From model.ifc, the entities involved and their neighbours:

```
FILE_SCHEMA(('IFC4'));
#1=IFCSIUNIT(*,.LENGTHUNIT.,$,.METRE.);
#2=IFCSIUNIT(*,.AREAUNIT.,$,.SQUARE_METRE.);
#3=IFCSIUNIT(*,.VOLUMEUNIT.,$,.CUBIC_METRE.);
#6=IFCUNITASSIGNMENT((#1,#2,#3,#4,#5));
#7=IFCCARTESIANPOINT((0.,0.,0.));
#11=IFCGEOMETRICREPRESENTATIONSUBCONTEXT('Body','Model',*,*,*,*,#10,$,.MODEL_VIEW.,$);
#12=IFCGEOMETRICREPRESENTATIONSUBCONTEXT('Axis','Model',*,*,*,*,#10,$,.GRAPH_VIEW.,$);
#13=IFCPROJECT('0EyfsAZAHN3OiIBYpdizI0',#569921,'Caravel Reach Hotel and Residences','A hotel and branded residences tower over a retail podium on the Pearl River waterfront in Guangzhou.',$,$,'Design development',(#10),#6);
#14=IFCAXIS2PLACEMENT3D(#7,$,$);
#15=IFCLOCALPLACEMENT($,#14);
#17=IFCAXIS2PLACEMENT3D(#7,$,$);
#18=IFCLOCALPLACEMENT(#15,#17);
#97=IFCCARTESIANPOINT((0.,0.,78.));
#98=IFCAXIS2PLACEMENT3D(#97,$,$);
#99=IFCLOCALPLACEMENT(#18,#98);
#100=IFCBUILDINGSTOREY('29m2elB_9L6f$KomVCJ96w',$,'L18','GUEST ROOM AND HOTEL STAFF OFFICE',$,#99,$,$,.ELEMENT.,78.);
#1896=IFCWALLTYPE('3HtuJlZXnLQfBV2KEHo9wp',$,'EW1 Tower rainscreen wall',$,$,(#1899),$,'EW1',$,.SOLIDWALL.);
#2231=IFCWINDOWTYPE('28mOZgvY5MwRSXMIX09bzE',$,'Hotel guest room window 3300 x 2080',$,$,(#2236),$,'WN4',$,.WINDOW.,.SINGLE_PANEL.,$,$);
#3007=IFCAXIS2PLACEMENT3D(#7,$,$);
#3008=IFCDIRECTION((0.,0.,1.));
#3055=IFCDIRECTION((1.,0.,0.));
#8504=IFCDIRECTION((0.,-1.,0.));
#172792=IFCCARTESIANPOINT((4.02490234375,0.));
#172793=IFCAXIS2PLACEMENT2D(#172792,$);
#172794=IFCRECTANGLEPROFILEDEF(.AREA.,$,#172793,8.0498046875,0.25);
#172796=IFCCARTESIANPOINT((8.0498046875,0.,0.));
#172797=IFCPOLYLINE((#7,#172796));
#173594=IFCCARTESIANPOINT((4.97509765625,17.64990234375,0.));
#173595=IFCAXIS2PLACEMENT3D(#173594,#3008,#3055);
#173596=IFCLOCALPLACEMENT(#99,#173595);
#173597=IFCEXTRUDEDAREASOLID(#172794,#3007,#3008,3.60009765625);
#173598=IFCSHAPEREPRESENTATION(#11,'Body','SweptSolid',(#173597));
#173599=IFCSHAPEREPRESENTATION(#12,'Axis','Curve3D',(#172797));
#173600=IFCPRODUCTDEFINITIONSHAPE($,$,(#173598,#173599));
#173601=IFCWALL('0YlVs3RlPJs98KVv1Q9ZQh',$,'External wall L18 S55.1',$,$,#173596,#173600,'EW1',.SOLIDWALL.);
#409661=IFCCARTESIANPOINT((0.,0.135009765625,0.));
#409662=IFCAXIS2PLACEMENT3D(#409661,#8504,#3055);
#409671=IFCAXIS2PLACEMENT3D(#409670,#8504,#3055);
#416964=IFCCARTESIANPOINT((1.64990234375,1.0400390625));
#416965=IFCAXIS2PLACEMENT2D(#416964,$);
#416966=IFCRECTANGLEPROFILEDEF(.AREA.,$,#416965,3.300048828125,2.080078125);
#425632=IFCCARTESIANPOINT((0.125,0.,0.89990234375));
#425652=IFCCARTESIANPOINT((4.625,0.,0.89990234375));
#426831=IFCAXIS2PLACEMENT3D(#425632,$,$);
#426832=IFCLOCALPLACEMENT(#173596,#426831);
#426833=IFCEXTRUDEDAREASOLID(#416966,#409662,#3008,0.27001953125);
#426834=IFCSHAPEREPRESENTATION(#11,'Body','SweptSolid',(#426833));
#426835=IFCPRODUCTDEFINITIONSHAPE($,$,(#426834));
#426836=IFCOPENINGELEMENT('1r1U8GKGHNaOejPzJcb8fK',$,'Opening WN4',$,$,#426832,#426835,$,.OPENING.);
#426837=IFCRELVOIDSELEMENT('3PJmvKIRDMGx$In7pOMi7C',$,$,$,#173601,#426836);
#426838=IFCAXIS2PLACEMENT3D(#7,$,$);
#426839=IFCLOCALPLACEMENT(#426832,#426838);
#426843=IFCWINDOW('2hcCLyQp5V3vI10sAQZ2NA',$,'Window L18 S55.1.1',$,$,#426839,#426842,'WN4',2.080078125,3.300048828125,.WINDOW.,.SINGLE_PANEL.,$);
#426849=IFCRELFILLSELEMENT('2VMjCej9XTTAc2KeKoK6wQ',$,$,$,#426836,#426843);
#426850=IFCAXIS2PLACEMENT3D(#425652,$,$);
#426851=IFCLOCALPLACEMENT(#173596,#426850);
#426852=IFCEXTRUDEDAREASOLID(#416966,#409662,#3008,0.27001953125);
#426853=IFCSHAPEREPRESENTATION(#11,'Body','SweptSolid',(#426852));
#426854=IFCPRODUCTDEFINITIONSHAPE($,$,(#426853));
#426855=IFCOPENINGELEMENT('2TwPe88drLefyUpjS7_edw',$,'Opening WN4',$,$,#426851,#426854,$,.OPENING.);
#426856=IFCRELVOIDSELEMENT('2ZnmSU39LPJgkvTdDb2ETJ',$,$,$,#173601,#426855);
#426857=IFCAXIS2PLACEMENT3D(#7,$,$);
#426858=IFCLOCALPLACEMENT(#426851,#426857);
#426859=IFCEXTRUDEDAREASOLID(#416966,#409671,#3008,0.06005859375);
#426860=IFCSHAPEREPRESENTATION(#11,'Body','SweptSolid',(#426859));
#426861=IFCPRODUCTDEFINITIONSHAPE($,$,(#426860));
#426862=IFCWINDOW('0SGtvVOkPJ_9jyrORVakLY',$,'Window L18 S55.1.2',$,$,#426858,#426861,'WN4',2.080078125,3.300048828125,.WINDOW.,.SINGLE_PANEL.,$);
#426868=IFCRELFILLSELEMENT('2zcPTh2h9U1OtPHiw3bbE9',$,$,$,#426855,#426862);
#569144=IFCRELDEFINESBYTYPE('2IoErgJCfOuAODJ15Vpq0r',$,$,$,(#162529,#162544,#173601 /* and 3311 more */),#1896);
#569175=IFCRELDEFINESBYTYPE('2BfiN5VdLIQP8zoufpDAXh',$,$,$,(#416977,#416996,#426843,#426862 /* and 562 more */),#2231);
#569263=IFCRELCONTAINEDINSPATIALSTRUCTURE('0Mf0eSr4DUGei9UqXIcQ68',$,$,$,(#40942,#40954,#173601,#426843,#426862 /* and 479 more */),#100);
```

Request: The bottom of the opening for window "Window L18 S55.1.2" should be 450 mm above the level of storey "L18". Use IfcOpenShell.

```python
import numpy as np
import ifcopenshell
import ifcopenshell.api.geometry
import ifcopenshell.geom
import ifcopenshell.util.element
import ifcopenshell.util.placement
import ifcopenshell.util.shape
import ifcopenshell.util.unit

model = ifcopenshell.open("model.ifc")
unit_scale = ifcopenshell.util.unit.calculate_unit_scale(model)

window = model.by_guid("0SGtvVOkPJ_9jyrORVakLY")
opening = window.FillsVoids[0].RelatingOpeningElement
storey = ifcopenshell.util.element.get_container(window, ifc_class="IfcBuildingStorey")
level = ifcopenshell.util.placement.get_local_placement(storey.ObjectPlacement)[2, 3]

# The opening's origin need not be at the sill, so measure its lowest point.
shape = ifcopenshell.geom.create_shape(ifcopenshell.geom.settings(), opening)
bottom = ifcopenshell.util.shape.get_shape_bottom_elevation(shape, shape.geometry) / unit_scale
dz = level + 0.45 - bottom

shift = np.array([0.0, 0.0, dz])
# The window is placed relative to its opening, so it follows when the opening moves.
matrix = ifcopenshell.util.placement.get_local_placement(opening.ObjectPlacement)
matrix[:3, 3] += shift
ifcopenshell.api.geometry.edit_object_placement(
    model, product=opening, matrix=matrix, is_si=False, should_transform_children=True
)

print(f"moved by {dz * unit_scale:+.3f} m")

model.write("model_rev.ifc")
```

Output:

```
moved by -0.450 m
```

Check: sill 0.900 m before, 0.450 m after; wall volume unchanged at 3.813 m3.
